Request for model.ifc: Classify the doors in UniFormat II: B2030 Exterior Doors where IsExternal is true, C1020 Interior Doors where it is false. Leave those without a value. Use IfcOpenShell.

First a look at what the model holds.

```python
import ifcopenshell
import ifcopenshell.util.element

model = ifcopenshell.open("model.ifc")
print(model.schema)
print("classifications:", [c.Name for c in model.by_type("IfcClassification")])
values = [ifcopenshell.util.element.get_pset(e, "Pset_DoorCommon", "IsExternal") for e in model.by_type("IfcDoor")]
for value in (True, False, None):
    print("IsExternal", value, values.count(value))
```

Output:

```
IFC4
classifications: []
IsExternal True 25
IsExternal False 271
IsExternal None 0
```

```python
import ifcopenshell
import ifcopenshell.api.classification
import ifcopenshell.util.element

model = ifcopenshell.open("model.ifc")

system = ifcopenshell.api.classification.add_classification(model, classification="UniFormat II")

doors = model.by_type("IfcDoor")
external = {e: ifcopenshell.util.element.get_pset(e, "Pset_DoorCommon", "IsExternal") for e in doors}
for flag, code, name in ((True, "B2030", "Exterior Doors"), (False, "C1020", "Interior Doors")):
    products = [e for e in doors if external[e] is flag]
    ifcopenshell.api.classification.add_reference(
        model, products=products, classification=system, identification=code, name=name
    )
    print(code, len(products))

model.write("model_v2.ifc")
```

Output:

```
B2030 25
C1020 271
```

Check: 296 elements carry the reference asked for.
